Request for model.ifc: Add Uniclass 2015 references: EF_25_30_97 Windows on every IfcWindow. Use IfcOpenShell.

First a look at what the model holds.

```python
import ifcopenshell

model = ifcopenshell.open("model.ifc")
print(model.schema)
print("classifications:", [c.Name for c in model.by_type("IfcClassification")])
for ifc_class in ("IfcDoor", "IfcRoof", "IfcStair", "IfcWall", "IfcWindow"):
    print(ifc_class, len(model.by_type(ifc_class)))
```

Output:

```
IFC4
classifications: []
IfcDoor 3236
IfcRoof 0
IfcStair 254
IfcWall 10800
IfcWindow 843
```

```python
import ifcopenshell
import ifcopenshell.api.classification

model = ifcopenshell.open("model.ifc")

system = ifcopenshell.api.classification.add_classification(model, classification="Uniclass 2015")

codes = {
    "IfcWindow": ("EF_25_30_97", "Windows"),
}
for ifc_class, (code, name) in codes.items():
    products = model.by_type(ifc_class)
    ifcopenshell.api.classification.add_reference(
        model, products=products, classification=system, identification=code, name=name
    )
    print(code, len(products))

model.write("model_edited.ifc")
```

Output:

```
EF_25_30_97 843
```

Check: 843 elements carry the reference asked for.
